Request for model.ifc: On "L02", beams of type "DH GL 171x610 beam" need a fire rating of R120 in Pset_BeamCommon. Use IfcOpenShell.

First a look at what the model holds.

```python
import ifcopenshell
import ifcopenshell.util.element

model = ifcopenshell.open("model.ifc")
print(model.schema)
storey = next(s for s in model.by_type("IfcBuildingStorey") if s.Name == "L02")
beams = [e for e in ifcopenshell.util.element.get_decomposition(storey) if e.is_a("IfcBeam")]
seen = {}
for e in beams:
    element_type = ifcopenshell.util.element.get_type(e)
    key = (element_type.Name if element_type != e and element_type else None, ifcopenshell.util.element.get_pset(e, "Pset_BeamCommon", "FireRating"))
    seen[key] = seen.get(key, 0) + 1
for (name, value), count in sorted(seen.items(), key=str):
    print(count, "x", name, "|", value)
```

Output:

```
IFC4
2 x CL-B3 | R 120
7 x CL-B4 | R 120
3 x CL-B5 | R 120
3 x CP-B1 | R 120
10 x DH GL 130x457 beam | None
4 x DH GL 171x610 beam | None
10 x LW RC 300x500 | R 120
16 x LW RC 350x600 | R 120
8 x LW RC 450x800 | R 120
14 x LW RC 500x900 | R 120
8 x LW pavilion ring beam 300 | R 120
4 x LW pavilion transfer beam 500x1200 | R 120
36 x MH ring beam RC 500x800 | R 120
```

```python
import ifcopenshell
import ifcopenshell.api.pset
import ifcopenshell.util.element

model = ifcopenshell.open("model.ifc")

storey = next(s for s in model.by_type("IfcBuildingStorey") if s.Name == "L02")
beams = [e for e in ifcopenshell.util.element.get_decomposition(storey) if e.is_a("IfcBeam")]

count = 0
for e in beams:
    element_type = ifcopenshell.util.element.get_type(e)
    if element_type in (None, e) or element_type.Name != "DH GL 171x610 beam":
        continue
    # add_pset returns the element's existing set when there is one.
    pset = ifcopenshell.api.pset.add_pset(model, product=e, name="Pset_BeamCommon")
    ifcopenshell.api.pset.edit_pset(model, pset=pset, properties={"FireRating": "R120"})
    count += 1

print(count, "beams updated")

model.write("model_rev.ifc")
```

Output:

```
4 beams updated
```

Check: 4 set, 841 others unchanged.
